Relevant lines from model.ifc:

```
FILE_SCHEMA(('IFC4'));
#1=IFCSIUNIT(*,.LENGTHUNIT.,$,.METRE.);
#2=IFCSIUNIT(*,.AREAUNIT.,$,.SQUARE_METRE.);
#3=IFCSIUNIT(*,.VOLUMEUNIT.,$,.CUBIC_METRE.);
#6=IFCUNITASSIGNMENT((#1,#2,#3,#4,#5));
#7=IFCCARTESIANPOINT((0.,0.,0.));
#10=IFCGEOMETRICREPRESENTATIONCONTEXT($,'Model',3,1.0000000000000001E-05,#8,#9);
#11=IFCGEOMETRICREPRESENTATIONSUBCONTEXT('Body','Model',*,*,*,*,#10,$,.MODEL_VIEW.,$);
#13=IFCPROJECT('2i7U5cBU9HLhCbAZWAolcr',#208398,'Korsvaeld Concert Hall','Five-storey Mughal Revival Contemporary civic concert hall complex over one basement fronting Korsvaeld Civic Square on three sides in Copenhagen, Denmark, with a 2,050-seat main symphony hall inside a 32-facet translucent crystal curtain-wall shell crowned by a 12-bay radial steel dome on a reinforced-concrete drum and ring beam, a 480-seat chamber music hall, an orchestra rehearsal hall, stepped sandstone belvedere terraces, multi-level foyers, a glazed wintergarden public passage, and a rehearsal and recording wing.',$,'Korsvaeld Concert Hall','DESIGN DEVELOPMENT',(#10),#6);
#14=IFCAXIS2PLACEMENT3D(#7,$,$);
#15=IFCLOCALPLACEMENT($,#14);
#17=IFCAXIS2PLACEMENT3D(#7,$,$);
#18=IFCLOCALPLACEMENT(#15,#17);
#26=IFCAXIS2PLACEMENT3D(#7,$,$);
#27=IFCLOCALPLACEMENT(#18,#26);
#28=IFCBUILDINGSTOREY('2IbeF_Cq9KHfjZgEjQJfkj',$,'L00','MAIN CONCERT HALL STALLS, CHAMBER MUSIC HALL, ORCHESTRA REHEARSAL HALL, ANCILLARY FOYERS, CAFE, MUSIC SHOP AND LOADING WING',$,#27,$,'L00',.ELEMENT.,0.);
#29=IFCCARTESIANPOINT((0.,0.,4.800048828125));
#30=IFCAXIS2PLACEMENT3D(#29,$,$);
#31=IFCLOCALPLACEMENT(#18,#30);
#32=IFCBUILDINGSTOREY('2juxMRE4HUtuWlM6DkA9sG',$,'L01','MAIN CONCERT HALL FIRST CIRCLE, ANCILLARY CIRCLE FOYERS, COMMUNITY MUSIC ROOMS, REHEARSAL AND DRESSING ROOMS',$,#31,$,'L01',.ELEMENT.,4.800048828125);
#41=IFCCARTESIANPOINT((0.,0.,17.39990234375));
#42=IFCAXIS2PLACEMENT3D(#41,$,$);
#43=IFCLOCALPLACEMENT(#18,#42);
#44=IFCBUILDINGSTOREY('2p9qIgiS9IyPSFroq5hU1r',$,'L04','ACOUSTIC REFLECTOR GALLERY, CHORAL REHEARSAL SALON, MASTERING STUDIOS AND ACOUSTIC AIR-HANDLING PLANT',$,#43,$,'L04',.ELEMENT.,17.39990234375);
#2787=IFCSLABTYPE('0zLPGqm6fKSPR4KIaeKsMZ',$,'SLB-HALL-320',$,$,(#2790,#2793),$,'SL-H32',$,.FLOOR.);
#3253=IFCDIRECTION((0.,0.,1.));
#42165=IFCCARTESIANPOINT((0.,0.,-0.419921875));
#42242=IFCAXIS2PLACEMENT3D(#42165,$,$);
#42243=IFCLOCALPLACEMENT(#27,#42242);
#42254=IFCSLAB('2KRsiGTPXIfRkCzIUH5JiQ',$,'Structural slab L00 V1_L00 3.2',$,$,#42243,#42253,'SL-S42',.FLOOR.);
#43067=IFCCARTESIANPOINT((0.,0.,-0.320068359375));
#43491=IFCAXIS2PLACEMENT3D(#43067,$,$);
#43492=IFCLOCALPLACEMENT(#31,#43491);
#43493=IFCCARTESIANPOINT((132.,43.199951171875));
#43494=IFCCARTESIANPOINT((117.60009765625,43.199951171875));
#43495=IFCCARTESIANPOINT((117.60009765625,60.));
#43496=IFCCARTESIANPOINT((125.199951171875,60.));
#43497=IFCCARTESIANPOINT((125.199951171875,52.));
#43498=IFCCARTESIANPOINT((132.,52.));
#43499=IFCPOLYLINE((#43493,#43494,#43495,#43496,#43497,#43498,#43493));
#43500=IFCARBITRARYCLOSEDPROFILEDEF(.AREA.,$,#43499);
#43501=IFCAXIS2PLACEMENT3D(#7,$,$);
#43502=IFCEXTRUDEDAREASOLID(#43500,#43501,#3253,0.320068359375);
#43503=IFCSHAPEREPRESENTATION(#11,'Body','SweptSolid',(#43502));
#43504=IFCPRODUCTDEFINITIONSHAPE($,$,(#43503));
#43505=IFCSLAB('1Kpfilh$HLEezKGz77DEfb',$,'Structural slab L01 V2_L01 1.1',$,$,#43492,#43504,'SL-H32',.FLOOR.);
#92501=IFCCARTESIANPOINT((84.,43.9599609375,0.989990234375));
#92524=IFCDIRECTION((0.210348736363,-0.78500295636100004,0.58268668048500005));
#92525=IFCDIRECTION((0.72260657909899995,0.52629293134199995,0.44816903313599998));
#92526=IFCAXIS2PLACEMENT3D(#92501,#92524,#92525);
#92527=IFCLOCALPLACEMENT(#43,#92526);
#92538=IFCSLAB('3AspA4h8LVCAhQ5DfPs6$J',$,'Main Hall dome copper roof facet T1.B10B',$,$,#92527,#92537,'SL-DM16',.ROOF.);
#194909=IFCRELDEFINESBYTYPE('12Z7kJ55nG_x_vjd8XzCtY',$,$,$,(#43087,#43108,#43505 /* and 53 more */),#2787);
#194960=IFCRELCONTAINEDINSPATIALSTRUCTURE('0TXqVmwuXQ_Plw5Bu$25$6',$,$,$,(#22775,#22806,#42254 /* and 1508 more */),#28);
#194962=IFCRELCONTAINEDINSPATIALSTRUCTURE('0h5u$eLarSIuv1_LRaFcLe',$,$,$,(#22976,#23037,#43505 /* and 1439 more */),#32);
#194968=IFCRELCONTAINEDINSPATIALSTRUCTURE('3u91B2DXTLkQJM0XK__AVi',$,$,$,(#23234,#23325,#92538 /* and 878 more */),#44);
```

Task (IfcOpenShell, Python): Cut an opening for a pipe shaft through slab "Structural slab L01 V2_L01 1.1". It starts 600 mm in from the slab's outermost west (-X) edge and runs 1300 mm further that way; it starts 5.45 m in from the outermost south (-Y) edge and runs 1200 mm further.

```python
import numpy as np
import ifcopenshell
import ifcopenshell.api.feature
import ifcopenshell.api.geometry
import ifcopenshell.api.root
import ifcopenshell.geom
import ifcopenshell.util.placement
import ifcopenshell.util.representation
import ifcopenshell.util.shape
import ifcopenshell.util.unit

model = ifcopenshell.open("model.ifc")
unit_scale = ifcopenshell.util.unit.calculate_unit_scale(model)
settings = ifcopenshell.geom.settings()


def volume(element):
    """Net volume in cubic metres, openings subtracted."""
    shape = ifcopenshell.geom.create_shape(settings, element)
    return ifcopenshell.util.shape.get_volume(shape.geometry)


slab = model.by_id(43505)
before = volume(slab)

# Extent in the slab's own axes, in metres. The edges named are its -X and -Y sides.
slab_shape = ifcopenshell.geom.create_shape(settings, slab)
vertices = ifcopenshell.util.shape.get_vertices(slab_shape.geometry)
x_min, y_min, bottom = vertices.min(axis=0)
top = vertices[:, 2].max()

opening = ifcopenshell.api.root.create_entity(model, ifc_class="IfcOpeningElement", name="Pipe shaft opening", predefined_type="OPENING")
context = ifcopenshell.util.representation.get_context(model, "Model", "Body", "MODEL_VIEW")
width, depth = 1.3, 1.2
outline = [(0.0, 0.0), (width, 0.0), (width, depth), (0.0, depth), (0.0, 0.0)]
# Overshoot both faces by 50 mm so the cut is clean.
shape = ifcopenshell.api.geometry.add_slab_representation(
    model, context=context, depth=top - bottom + 0.1, polyline=outline
)
ifcopenshell.api.geometry.assign_representation(model, product=opening, representation=shape)

matrix = ifcopenshell.util.placement.get_local_placement(slab.ObjectPlacement)
matrix[:, 3] = matrix @ np.append(np.array([x_min + 0.6, y_min + 5.45, bottom - 0.05]) / unit_scale, 1.0)
ifcopenshell.api.geometry.edit_object_placement(model, product=opening, matrix=matrix, is_si=False)
ifcopenshell.api.feature.add_feature(model, feature=opening, element=slab)

after = volume(slab)

print(f"slab volume {before:.3f} -> {after:.3f} m3")

model.write("model_v2.ifc")
```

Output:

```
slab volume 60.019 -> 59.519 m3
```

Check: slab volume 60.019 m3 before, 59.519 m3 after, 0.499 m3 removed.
